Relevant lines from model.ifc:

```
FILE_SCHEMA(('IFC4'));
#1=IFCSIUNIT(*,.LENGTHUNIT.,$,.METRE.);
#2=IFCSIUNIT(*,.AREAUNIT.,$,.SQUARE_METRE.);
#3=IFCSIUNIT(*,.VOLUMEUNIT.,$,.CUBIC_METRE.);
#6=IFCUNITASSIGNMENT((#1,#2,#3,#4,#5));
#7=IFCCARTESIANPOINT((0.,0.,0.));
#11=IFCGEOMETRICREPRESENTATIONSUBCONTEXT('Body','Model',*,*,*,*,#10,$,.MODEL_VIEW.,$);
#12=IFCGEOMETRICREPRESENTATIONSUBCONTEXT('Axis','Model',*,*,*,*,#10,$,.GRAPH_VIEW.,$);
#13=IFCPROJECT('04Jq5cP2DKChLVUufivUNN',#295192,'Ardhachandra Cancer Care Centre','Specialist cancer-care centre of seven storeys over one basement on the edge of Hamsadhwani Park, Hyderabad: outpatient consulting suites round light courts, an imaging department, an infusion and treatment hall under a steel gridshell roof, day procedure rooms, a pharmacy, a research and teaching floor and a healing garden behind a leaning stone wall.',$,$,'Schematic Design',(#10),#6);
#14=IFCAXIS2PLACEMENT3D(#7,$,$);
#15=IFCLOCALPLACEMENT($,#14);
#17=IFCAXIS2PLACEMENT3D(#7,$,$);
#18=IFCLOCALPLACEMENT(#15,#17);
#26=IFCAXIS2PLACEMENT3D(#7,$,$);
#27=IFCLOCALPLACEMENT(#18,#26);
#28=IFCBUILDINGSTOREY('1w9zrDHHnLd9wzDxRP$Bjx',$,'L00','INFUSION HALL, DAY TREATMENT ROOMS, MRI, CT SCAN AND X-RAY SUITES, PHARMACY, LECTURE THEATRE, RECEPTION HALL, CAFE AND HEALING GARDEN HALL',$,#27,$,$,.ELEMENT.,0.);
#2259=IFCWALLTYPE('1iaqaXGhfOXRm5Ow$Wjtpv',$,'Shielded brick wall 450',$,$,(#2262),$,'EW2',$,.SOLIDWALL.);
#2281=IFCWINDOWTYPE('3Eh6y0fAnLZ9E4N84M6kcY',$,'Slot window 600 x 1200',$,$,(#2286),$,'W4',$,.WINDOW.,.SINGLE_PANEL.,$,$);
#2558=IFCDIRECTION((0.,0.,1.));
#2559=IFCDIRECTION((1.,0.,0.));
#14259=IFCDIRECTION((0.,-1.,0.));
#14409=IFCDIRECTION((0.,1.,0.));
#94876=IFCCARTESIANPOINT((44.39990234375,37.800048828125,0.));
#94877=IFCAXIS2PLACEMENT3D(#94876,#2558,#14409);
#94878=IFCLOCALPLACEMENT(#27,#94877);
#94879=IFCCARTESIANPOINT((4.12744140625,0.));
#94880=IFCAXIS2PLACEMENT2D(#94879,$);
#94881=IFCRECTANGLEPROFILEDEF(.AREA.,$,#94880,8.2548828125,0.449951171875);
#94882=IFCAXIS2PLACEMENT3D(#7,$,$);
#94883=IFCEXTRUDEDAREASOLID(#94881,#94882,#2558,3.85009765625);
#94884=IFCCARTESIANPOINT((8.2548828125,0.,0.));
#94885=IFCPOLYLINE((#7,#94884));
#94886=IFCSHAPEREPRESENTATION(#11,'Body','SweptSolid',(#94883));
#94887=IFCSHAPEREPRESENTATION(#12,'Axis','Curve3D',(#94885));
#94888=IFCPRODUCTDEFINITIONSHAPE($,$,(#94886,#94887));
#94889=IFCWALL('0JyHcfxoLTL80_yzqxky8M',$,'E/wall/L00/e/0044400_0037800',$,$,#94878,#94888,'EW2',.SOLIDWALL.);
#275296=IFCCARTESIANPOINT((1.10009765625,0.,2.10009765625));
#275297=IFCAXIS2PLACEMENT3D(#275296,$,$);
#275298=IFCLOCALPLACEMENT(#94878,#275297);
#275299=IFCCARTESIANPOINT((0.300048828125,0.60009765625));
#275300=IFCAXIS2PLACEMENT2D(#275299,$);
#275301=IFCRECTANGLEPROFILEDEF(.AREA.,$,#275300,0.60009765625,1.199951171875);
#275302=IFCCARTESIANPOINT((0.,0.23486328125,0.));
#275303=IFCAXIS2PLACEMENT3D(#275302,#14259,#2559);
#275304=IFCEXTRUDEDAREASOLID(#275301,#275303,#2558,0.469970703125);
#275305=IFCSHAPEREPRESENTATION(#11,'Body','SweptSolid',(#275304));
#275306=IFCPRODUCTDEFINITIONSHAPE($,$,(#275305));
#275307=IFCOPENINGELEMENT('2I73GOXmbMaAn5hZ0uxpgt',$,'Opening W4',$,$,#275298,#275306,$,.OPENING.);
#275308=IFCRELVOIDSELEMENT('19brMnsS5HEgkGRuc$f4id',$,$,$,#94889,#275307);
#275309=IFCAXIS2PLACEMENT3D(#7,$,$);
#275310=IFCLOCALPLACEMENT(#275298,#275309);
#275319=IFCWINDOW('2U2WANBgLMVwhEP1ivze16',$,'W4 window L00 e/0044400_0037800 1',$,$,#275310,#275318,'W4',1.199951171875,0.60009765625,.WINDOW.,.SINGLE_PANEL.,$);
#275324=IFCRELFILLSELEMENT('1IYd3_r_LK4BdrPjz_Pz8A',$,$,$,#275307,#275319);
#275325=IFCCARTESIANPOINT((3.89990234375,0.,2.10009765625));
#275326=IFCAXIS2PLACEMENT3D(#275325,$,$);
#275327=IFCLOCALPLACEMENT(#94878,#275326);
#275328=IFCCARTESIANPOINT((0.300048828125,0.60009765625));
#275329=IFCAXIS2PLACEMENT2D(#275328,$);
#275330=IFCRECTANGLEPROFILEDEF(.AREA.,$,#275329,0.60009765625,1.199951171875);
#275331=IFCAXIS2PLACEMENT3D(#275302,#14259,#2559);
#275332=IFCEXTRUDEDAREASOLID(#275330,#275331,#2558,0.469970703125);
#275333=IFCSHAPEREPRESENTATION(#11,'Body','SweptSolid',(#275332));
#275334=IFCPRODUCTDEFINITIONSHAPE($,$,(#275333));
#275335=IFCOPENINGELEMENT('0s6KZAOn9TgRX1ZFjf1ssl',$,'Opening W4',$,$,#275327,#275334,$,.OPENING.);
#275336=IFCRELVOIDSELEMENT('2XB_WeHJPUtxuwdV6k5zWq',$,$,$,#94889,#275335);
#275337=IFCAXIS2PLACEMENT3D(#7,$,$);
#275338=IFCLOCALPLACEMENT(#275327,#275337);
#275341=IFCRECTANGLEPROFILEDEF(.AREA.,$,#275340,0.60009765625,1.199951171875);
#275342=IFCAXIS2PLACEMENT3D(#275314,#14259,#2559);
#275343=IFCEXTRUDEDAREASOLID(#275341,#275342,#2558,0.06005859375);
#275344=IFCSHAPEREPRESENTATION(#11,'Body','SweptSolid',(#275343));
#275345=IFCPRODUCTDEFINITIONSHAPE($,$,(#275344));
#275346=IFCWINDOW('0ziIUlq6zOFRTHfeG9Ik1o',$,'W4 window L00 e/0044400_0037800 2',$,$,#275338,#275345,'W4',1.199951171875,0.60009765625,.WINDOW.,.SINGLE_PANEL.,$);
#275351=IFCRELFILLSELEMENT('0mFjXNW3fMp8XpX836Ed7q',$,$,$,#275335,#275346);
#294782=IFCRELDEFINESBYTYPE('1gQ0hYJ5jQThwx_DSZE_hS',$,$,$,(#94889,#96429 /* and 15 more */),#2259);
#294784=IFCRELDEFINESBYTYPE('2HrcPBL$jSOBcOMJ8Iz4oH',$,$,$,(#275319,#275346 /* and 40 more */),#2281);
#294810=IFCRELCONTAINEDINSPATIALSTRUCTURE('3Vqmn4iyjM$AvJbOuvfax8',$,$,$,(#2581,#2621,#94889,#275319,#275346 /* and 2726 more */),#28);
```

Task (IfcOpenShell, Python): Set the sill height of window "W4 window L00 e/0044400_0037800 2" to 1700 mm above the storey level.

```python
import numpy as np
import ifcopenshell
import ifcopenshell.api.geometry
import ifcopenshell.geom
import ifcopenshell.util.element
import ifcopenshell.util.placement
import ifcopenshell.util.shape
import ifcopenshell.util.unit

model = ifcopenshell.open("model.ifc")
unit_scale = ifcopenshell.util.unit.calculate_unit_scale(model)

window = model.by_id(275346)
opening = window.FillsVoids[0].RelatingOpeningElement
storey = ifcopenshell.util.element.get_container(window, ifc_class="IfcBuildingStorey")
level = ifcopenshell.util.placement.get_local_placement(storey.ObjectPlacement)[2, 3]

# The opening's origin need not be at the sill, so measure its lowest point.
shape = ifcopenshell.geom.create_shape(ifcopenshell.geom.settings(), opening)
bottom = ifcopenshell.util.shape.get_shape_bottom_elevation(shape, shape.geometry) / unit_scale
dz = level + 1.7 - bottom

shift = np.array([0.0, 0.0, dz])
# The window is placed relative to its opening, so it follows when the opening moves.
matrix = ifcopenshell.util.placement.get_local_placement(opening.ObjectPlacement)
matrix[:3, 3] += shift
ifcopenshell.api.geometry.edit_object_placement(
    model, product=opening, matrix=matrix, is_si=False, should_transform_children=True
)

print(f"moved by {dz * unit_scale:+.3f} m")

model.write("model_updated.ifc")
```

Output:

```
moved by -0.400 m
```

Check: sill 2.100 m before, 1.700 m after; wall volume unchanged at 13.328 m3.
